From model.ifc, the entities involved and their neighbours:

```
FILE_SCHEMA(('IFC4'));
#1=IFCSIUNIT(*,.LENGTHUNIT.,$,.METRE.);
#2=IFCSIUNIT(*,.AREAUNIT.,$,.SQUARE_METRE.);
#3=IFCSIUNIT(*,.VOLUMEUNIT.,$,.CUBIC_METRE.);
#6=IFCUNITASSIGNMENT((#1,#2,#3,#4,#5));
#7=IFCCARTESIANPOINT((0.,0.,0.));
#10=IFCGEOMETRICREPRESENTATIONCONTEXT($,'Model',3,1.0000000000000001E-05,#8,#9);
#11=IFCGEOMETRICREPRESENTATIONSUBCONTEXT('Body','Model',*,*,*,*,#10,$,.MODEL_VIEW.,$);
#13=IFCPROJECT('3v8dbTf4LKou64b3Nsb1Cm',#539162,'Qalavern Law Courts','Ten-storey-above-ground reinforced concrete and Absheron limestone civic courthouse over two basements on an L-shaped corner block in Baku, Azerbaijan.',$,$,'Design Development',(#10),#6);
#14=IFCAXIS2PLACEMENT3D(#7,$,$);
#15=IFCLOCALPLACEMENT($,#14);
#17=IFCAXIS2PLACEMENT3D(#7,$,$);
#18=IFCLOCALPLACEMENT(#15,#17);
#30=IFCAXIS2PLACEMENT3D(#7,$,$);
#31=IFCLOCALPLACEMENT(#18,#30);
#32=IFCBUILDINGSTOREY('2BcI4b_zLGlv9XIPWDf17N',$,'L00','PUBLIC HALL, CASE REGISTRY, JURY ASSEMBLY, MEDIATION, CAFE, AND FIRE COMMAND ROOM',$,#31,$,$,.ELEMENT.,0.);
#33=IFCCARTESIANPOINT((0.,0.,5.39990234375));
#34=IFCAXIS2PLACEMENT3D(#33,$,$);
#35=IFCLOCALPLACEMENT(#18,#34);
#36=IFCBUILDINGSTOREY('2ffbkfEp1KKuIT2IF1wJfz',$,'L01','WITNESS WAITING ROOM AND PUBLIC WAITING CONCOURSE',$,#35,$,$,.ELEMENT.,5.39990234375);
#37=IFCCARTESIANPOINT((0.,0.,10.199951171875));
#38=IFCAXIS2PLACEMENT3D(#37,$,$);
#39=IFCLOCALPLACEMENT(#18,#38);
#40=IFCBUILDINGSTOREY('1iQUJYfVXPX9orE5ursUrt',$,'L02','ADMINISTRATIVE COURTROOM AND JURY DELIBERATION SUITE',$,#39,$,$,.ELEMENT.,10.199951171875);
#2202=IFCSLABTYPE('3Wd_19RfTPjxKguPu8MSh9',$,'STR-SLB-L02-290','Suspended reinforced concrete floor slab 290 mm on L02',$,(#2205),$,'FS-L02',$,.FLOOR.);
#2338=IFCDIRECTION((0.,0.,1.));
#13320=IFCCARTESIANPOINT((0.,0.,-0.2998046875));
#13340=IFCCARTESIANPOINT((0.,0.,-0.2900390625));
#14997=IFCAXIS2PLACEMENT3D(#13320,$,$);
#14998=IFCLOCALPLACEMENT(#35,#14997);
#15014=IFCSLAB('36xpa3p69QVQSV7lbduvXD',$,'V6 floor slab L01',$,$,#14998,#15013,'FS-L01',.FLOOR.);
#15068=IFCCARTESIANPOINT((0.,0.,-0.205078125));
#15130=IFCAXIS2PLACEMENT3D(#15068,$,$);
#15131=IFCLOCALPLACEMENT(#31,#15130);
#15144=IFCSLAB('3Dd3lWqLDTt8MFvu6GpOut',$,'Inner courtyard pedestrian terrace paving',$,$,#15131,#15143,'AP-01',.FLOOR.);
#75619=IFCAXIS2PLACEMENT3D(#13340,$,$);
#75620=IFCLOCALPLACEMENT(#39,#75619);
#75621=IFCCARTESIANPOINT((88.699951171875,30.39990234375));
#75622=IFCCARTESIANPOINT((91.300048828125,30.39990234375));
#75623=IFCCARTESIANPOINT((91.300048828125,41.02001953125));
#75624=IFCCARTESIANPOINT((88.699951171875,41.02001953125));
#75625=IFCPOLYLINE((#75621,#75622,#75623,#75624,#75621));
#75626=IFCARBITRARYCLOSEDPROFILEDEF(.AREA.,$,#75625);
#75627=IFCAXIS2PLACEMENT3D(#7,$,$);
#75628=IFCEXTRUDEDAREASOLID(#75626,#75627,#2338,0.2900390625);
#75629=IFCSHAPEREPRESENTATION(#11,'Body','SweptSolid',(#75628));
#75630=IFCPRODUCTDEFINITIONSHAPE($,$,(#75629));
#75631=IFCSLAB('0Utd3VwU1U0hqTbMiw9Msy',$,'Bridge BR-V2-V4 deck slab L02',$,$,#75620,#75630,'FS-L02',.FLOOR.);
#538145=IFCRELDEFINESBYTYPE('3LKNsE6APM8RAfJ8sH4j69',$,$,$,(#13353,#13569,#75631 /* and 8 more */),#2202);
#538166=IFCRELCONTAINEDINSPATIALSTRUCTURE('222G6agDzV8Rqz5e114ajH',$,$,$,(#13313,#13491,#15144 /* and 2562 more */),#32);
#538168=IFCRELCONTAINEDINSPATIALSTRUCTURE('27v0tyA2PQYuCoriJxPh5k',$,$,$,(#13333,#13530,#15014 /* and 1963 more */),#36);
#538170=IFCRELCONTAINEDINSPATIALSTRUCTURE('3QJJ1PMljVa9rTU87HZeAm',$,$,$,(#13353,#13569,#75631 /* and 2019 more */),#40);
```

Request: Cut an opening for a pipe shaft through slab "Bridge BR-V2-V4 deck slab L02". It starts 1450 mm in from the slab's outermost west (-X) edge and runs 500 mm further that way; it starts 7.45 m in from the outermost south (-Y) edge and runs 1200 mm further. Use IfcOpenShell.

```python
import numpy as np
import ifcopenshell
import ifcopenshell.api.feature
import ifcopenshell.api.geometry
import ifcopenshell.api.root
import ifcopenshell.geom
import ifcopenshell.util.placement
import ifcopenshell.util.representation
import ifcopenshell.util.shape
import ifcopenshell.util.unit

model = ifcopenshell.open("model.ifc")
unit_scale = ifcopenshell.util.unit.calculate_unit_scale(model)
settings = ifcopenshell.geom.settings()


def volume(element):
    """Net volume in cubic metres, openings subtracted."""
    shape = ifcopenshell.geom.create_shape(settings, element)
    return ifcopenshell.util.shape.get_volume(shape.geometry)


slab = model.by_id(75631)
before = volume(slab)

# Extent in the slab's own axes, in metres. The edges named are its -X and -Y sides.
slab_shape = ifcopenshell.geom.create_shape(settings, slab)
vertices = ifcopenshell.util.shape.get_vertices(slab_shape.geometry)
x_min, y_min, bottom = vertices.min(axis=0)
top = vertices[:, 2].max()

opening = ifcopenshell.api.root.create_entity(model, ifc_class="IfcOpeningElement", name="Pipe shaft opening", predefined_type="OPENING")
context = ifcopenshell.util.representation.get_context(model, "Model", "Body", "MODEL_VIEW")
width, depth = 0.5, 1.2
outline = [(0.0, 0.0), (width, 0.0), (width, depth), (0.0, depth), (0.0, 0.0)]
# Overshoot both faces by 50 mm so the cut is clean.
shape = ifcopenshell.api.geometry.add_slab_representation(
    model, context=context, depth=top - bottom + 0.1, polyline=outline
)
ifcopenshell.api.geometry.assign_representation(model, product=opening, representation=shape)

matrix = ifcopenshell.util.placement.get_local_placement(slab.ObjectPlacement)
matrix[:, 3] = matrix @ np.append(np.array([x_min + 1.45, y_min + 7.45, bottom - 0.05]) / unit_scale, 1.0)
ifcopenshell.api.geometry.edit_object_placement(model, product=opening, matrix=matrix, is_si=False)
ifcopenshell.api.feature.add_feature(model, feature=opening, element=slab)

after = volume(slab)

print(f"slab volume {before:.3f} -> {after:.3f} m3")

model.write("model_updated.ifc")
```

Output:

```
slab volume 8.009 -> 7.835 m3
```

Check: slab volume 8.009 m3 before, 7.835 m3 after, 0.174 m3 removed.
